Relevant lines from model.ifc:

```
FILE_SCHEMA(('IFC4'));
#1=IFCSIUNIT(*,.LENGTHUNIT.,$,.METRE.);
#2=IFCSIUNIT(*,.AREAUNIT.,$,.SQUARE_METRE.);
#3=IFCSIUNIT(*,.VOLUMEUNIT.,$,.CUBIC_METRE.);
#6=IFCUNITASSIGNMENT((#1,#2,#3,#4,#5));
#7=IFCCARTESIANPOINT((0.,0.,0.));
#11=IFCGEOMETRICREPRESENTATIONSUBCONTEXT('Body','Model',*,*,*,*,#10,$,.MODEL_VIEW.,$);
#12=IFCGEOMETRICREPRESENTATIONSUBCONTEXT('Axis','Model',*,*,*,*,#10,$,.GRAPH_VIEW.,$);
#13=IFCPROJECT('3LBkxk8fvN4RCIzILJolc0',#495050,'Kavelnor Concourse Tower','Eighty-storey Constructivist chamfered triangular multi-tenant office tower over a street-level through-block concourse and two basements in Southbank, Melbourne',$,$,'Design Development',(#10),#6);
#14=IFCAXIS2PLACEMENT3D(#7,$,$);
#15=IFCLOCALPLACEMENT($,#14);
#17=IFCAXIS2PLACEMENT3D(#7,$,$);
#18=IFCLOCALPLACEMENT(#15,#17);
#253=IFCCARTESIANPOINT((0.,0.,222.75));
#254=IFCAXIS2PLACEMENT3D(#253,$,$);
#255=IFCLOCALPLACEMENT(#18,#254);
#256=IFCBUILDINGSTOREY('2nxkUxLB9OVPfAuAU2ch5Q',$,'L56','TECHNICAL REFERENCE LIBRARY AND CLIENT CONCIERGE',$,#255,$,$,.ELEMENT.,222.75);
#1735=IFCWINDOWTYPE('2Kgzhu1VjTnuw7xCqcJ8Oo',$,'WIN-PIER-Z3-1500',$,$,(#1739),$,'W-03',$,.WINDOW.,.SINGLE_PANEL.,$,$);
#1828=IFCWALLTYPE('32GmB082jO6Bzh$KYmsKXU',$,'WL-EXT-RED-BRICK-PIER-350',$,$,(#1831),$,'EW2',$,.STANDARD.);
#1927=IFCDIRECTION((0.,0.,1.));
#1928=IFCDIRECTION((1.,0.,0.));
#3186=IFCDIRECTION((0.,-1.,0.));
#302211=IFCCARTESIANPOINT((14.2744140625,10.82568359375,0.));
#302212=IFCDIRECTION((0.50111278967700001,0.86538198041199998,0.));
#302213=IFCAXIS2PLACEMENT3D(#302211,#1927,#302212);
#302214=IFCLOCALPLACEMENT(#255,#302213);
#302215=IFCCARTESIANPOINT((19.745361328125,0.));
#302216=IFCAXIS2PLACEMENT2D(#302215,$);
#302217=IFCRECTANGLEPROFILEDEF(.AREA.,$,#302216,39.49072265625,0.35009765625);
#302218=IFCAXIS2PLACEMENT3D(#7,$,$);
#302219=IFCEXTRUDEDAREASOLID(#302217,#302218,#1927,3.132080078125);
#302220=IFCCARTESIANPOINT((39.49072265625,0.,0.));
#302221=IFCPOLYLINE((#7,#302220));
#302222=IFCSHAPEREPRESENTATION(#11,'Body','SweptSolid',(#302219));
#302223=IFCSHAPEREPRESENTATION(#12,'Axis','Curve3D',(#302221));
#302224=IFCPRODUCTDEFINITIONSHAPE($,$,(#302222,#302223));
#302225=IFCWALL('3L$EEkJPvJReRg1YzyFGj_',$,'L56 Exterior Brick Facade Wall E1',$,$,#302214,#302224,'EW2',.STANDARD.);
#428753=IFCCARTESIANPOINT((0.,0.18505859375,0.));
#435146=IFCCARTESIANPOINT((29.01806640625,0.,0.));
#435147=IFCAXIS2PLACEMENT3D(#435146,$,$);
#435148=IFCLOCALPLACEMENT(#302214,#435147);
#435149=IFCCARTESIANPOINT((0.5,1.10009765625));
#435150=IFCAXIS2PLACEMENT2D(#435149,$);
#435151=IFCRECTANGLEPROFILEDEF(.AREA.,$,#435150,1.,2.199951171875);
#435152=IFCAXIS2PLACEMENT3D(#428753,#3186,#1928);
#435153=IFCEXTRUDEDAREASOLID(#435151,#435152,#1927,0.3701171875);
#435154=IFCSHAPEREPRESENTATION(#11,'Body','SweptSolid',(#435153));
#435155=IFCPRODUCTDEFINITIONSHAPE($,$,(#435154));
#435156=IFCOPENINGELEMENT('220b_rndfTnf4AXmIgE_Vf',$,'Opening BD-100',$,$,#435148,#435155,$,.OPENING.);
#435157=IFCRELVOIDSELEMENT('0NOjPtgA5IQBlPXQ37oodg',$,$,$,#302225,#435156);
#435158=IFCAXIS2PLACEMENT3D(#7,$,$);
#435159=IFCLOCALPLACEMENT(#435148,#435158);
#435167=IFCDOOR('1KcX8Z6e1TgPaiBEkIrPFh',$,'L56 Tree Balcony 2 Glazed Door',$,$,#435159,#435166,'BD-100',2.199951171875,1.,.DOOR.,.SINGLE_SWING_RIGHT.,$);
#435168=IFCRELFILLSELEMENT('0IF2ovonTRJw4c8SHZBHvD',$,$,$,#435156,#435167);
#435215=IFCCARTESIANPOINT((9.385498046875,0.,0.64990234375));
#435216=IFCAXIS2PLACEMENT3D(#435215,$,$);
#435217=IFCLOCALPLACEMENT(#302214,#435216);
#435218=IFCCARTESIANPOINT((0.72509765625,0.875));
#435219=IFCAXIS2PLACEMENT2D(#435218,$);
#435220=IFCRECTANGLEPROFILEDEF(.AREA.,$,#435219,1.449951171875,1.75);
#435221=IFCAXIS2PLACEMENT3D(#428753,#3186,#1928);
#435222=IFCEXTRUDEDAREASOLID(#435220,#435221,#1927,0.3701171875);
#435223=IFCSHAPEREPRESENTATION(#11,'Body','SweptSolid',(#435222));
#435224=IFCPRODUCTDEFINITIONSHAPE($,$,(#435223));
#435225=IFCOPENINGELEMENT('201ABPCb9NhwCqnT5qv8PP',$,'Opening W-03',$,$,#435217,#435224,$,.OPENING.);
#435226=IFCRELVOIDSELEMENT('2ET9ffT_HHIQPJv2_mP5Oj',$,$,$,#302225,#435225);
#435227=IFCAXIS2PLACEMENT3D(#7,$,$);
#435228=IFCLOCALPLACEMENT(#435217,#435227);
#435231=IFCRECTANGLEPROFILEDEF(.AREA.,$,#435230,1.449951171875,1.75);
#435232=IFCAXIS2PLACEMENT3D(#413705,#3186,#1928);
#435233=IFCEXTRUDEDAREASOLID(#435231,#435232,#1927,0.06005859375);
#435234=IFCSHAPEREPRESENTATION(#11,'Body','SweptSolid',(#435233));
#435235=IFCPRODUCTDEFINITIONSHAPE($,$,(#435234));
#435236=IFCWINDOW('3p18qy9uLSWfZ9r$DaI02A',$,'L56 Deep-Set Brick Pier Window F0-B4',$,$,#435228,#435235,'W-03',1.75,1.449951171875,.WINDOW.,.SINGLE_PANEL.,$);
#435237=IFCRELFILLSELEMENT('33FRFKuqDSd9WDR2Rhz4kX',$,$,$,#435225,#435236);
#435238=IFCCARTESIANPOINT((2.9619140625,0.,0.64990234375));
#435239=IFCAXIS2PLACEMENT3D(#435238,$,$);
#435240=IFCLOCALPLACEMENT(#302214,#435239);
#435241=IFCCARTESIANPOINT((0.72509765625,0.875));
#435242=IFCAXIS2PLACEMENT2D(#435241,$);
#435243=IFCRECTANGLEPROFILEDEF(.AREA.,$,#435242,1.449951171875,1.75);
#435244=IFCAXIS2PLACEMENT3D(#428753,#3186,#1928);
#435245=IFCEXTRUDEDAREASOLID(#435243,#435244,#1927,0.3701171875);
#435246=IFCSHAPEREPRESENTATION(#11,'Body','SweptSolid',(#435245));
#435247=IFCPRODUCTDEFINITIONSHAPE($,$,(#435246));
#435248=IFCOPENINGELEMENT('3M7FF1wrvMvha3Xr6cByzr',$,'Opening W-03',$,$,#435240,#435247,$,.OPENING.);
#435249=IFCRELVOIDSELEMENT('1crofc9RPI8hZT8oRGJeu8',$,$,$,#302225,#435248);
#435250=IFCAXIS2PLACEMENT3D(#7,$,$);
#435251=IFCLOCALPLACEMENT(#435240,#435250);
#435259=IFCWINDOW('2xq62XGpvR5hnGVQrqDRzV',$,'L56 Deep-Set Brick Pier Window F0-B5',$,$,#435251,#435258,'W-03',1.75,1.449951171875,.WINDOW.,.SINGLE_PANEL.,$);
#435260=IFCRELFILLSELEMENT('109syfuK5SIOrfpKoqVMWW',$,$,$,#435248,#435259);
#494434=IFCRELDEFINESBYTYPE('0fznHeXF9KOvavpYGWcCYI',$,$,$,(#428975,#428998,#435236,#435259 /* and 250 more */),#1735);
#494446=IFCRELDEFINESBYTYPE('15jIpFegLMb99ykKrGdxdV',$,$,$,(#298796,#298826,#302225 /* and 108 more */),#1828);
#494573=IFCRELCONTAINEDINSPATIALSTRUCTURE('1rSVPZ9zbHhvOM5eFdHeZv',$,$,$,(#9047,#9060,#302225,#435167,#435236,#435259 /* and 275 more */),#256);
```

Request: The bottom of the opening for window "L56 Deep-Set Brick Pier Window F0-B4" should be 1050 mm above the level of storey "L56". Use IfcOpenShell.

```python
import numpy as np
import ifcopenshell
import ifcopenshell.api.geometry
import ifcopenshell.geom
import ifcopenshell.util.element
import ifcopenshell.util.placement
import ifcopenshell.util.shape
import ifcopenshell.util.unit

model = ifcopenshell.open("model.ifc")
unit_scale = ifcopenshell.util.unit.calculate_unit_scale(model)

window = model.by_guid("3p18qy9uLSWfZ9r$DaI02A")
opening = window.FillsVoids[0].RelatingOpeningElement
storey = ifcopenshell.util.element.get_container(window, ifc_class="IfcBuildingStorey")
level = ifcopenshell.util.placement.get_local_placement(storey.ObjectPlacement)[2, 3]

# The opening's origin need not be at the sill, so measure its lowest point.
shape = ifcopenshell.geom.create_shape(ifcopenshell.geom.settings(), opening)
bottom = ifcopenshell.util.shape.get_shape_bottom_elevation(shape, shape.geometry) / unit_scale
dz = level + 1.05 / unit_scale - bottom

shift = np.array([0.0, 0.0, dz])
# The window is placed relative to its opening, so it follows when the opening moves.
matrix = ifcopenshell.util.placement.get_local_placement(opening.ObjectPlacement)
matrix[:3, 3] += shift
ifcopenshell.api.geometry.edit_object_placement(
    model, product=opening, matrix=matrix, is_si=False, should_transform_children=True
)

print(f"moved by {dz * unit_scale:+.3f} m")

model.write("model_v2.ifc")
```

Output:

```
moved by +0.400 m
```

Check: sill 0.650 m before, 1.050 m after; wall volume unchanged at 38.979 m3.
